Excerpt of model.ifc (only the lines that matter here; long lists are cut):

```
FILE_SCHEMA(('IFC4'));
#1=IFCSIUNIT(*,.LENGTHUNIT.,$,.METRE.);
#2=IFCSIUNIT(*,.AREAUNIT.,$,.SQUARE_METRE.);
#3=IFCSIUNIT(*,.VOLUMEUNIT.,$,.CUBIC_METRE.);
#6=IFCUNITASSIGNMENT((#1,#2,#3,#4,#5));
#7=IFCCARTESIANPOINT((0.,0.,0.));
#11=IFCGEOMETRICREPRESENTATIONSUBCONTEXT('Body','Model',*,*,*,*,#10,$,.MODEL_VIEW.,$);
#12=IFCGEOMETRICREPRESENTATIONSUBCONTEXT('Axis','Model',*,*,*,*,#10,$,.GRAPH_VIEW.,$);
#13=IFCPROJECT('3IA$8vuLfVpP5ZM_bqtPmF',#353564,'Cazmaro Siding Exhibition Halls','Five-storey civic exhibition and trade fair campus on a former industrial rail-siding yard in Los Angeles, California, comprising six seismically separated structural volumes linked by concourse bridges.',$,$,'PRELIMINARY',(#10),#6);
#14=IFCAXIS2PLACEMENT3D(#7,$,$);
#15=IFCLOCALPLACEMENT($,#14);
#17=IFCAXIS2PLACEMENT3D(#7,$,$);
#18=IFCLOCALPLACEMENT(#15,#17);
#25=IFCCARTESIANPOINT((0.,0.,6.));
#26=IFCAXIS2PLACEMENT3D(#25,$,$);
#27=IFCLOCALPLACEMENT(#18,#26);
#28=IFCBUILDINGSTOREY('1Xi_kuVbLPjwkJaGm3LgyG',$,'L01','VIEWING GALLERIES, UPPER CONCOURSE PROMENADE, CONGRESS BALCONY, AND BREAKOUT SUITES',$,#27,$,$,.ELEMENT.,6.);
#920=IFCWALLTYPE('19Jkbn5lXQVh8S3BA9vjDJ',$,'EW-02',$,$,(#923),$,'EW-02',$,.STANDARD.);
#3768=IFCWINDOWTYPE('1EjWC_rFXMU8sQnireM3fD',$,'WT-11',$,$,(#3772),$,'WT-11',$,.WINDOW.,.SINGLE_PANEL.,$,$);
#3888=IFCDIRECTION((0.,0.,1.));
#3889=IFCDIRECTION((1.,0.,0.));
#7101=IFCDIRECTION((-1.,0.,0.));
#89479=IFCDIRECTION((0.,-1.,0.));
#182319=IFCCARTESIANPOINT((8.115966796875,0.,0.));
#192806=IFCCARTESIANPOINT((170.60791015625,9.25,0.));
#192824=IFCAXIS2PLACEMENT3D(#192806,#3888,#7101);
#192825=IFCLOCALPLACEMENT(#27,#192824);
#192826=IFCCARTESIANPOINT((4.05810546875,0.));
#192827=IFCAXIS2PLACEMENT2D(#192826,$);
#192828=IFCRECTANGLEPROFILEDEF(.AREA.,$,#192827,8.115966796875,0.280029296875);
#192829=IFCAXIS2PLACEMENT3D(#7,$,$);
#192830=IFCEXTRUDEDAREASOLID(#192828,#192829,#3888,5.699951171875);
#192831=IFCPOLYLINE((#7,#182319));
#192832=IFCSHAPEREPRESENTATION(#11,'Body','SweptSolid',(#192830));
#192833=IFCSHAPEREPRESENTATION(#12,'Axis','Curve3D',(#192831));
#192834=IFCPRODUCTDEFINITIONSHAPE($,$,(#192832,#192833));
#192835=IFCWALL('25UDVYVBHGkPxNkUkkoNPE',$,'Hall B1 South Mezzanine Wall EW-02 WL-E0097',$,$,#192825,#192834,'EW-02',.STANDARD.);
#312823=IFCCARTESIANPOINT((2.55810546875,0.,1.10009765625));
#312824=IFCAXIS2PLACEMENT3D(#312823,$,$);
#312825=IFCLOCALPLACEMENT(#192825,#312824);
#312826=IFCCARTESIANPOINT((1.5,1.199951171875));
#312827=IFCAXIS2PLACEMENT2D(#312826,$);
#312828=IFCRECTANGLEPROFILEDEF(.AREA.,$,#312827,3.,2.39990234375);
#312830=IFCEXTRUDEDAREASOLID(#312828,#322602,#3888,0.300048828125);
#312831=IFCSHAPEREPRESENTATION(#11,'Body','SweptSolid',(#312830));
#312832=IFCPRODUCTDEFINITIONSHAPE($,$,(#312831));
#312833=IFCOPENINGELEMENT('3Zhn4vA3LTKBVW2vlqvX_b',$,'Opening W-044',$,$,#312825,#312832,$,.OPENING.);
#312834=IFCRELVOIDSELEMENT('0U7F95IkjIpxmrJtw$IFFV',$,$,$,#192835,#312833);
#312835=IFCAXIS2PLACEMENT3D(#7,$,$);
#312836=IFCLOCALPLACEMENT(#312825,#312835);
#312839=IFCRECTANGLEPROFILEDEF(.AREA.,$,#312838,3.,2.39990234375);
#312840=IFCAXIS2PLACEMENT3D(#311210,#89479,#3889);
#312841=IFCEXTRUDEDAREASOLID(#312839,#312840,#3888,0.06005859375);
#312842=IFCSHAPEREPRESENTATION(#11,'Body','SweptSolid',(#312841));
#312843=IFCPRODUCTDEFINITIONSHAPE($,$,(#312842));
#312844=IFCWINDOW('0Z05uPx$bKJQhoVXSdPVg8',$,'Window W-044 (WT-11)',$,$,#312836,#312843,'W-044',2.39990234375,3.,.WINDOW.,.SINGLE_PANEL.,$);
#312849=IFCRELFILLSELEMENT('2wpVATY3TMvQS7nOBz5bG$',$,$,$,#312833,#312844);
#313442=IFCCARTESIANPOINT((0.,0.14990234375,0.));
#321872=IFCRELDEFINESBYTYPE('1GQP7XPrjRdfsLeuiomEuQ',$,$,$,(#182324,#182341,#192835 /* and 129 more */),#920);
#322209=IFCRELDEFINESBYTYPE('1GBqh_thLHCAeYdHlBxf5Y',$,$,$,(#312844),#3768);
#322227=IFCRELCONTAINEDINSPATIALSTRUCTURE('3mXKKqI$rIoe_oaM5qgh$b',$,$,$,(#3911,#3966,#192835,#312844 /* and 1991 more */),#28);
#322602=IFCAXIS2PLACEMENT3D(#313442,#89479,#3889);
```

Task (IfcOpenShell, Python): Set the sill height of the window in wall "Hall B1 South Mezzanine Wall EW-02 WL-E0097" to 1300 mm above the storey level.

```python
import numpy as np
import ifcopenshell
import ifcopenshell.api.geometry
import ifcopenshell.geom
import ifcopenshell.util.element
import ifcopenshell.util.placement
import ifcopenshell.util.shape
import ifcopenshell.util.unit

model = ifcopenshell.open("model.ifc")
unit_scale = ifcopenshell.util.unit.calculate_unit_scale(model)

window = model.by_guid("0Z05uPx$bKJQhoVXSdPVg8")
opening = window.FillsVoids[0].RelatingOpeningElement
storey = ifcopenshell.util.element.get_container(window, ifc_class="IfcBuildingStorey")
level = ifcopenshell.util.placement.get_local_placement(storey.ObjectPlacement)[2, 3]

# The opening's origin need not be at the sill, so measure its lowest point.
shape = ifcopenshell.geom.create_shape(ifcopenshell.geom.settings(), opening)
bottom = ifcopenshell.util.shape.get_shape_bottom_elevation(shape, shape.geometry) / unit_scale
dz = level + 1.3 / unit_scale - bottom

shift = np.array([0.0, 0.0, dz])
# The window is placed relative to its opening, so it follows when the opening moves.
matrix = ifcopenshell.util.placement.get_local_placement(opening.ObjectPlacement)
matrix[:3, 3] += shift
ifcopenshell.api.geometry.edit_object_placement(
    model, product=opening, matrix=matrix, is_si=False, should_transform_children=True
)

print(f"moved by {dz * unit_scale:+.3f} m")

model.write("model_rev.ifc")
```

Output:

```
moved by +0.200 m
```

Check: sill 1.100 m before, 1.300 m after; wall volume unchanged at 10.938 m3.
